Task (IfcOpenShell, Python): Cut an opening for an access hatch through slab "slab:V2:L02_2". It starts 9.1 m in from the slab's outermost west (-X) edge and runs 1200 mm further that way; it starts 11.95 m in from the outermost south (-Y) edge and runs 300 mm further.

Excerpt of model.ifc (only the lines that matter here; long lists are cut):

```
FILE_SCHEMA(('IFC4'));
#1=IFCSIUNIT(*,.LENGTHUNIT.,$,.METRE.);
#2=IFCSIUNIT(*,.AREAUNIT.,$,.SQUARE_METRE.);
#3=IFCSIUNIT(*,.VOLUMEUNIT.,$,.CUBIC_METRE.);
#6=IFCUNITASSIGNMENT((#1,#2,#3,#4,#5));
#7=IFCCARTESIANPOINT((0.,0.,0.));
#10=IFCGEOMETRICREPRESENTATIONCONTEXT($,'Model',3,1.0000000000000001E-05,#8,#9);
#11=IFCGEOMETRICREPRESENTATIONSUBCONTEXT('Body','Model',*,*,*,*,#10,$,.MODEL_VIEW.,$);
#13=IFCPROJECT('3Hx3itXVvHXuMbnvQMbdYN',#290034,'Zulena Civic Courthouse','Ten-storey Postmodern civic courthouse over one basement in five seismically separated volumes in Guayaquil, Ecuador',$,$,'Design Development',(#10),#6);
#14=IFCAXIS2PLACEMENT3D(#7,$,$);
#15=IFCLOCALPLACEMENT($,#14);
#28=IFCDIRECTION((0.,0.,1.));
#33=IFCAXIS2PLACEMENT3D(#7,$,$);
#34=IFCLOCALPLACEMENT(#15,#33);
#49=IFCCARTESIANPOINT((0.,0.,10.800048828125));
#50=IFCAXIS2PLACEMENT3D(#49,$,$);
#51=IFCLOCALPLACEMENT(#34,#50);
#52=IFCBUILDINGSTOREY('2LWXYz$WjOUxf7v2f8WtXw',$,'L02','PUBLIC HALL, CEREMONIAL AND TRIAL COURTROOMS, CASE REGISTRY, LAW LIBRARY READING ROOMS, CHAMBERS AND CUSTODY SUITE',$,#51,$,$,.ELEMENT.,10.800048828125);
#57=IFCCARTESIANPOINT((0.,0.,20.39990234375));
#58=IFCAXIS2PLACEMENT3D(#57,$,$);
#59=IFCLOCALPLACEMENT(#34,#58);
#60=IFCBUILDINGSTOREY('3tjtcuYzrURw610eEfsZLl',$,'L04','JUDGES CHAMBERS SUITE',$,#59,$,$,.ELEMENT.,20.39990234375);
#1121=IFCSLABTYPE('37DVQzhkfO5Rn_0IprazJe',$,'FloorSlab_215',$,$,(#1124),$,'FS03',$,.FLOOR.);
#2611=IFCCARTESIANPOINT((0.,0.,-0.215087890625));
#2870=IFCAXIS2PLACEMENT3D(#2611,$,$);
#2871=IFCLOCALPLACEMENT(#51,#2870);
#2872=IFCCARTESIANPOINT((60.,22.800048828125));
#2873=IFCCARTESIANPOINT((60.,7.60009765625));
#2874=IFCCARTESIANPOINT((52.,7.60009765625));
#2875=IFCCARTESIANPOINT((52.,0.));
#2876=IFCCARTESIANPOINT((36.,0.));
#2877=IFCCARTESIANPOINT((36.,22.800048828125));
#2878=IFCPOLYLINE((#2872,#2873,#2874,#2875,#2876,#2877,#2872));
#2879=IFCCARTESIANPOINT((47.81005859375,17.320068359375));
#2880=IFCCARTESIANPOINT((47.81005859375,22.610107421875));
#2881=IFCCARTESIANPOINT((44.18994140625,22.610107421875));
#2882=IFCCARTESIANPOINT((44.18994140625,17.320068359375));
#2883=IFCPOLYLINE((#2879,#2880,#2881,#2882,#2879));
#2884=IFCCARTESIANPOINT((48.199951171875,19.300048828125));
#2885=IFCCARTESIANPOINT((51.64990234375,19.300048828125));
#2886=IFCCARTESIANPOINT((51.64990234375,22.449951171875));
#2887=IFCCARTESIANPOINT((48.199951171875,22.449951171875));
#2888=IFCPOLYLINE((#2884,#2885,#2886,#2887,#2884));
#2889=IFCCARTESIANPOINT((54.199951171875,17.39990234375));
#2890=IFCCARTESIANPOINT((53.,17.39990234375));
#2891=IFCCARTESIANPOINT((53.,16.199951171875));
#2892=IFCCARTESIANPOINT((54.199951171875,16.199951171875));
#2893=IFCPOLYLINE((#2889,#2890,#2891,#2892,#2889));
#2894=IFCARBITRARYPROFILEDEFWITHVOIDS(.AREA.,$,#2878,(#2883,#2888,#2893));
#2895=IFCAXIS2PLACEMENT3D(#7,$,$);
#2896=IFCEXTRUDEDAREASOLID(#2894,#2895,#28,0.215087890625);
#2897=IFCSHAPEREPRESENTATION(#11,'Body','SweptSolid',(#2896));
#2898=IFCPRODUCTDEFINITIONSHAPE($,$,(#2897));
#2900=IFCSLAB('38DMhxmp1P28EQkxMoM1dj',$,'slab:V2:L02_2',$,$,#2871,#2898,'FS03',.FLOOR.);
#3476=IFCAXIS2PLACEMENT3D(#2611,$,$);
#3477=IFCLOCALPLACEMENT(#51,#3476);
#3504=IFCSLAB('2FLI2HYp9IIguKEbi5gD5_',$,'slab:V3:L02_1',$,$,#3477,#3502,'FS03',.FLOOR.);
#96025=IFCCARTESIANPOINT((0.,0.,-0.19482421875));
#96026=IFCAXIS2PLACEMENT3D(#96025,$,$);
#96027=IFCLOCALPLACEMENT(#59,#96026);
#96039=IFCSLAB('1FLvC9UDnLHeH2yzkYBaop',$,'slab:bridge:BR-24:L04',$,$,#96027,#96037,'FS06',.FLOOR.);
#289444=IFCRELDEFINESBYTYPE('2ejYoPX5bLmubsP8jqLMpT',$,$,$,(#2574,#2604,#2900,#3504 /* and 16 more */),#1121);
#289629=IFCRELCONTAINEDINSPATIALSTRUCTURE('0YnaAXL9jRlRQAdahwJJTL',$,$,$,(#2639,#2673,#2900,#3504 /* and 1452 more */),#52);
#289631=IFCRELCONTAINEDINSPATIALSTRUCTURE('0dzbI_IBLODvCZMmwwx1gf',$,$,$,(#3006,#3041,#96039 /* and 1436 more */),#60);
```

```python
import numpy as np
import ifcopenshell
import ifcopenshell.api.feature
import ifcopenshell.api.geometry
import ifcopenshell.api.root
import ifcopenshell.geom
import ifcopenshell.util.placement
import ifcopenshell.util.representation
import ifcopenshell.util.shape
import ifcopenshell.util.unit

model = ifcopenshell.open("model.ifc")
unit_scale = ifcopenshell.util.unit.calculate_unit_scale(model)
settings = ifcopenshell.geom.settings()


def volume(element):
    """Net volume in cubic metres, openings subtracted."""
    shape = ifcopenshell.geom.create_shape(settings, element)
    return ifcopenshell.util.shape.get_volume(shape.geometry)


slab = model.by_guid("38DMhxmp1P28EQkxMoM1dj")
before = volume(slab)

# Extent in the slab's own axes, in metres. The edges named are its -X and -Y sides.
slab_shape = ifcopenshell.geom.create_shape(settings, slab)
vertices = ifcopenshell.util.shape.get_vertices(slab_shape.geometry)
x_min, y_min, bottom = vertices.min(axis=0)
top = vertices[:, 2].max()

opening = ifcopenshell.api.root.create_entity(model, ifc_class="IfcOpeningElement", name="Access hatch opening", predefined_type="OPENING")
context = ifcopenshell.util.representation.get_context(model, "Model", "Body", "MODEL_VIEW")
width, depth = 1.2, 0.3
outline = [(0.0, 0.0), (width, 0.0), (width, depth), (0.0, depth), (0.0, 0.0)]
# Overshoot both faces by 50 mm so the cut is clean.
shape = ifcopenshell.api.geometry.add_slab_representation(
    model, context=context, depth=top - bottom + 0.1, polyline=outline
)
ifcopenshell.api.geometry.assign_representation(model, product=opening, representation=shape)

matrix = ifcopenshell.util.placement.get_local_placement(slab.ObjectPlacement)
matrix[:, 3] = matrix @ np.append(np.array([x_min + 9.1, y_min + 11.95, bottom - 0.05]) / unit_scale, 1.0)
ifcopenshell.api.geometry.edit_object_placement(model, product=opening, matrix=matrix, is_si=False)
ifcopenshell.api.feature.add_feature(model, feature=opening, element=slab)

after = volume(slab)

print(f"slab volume {before:.3f} -> {after:.3f} m3")

model.write("model_rev.ifc")
```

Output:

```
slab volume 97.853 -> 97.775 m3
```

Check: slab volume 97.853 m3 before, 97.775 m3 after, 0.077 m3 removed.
